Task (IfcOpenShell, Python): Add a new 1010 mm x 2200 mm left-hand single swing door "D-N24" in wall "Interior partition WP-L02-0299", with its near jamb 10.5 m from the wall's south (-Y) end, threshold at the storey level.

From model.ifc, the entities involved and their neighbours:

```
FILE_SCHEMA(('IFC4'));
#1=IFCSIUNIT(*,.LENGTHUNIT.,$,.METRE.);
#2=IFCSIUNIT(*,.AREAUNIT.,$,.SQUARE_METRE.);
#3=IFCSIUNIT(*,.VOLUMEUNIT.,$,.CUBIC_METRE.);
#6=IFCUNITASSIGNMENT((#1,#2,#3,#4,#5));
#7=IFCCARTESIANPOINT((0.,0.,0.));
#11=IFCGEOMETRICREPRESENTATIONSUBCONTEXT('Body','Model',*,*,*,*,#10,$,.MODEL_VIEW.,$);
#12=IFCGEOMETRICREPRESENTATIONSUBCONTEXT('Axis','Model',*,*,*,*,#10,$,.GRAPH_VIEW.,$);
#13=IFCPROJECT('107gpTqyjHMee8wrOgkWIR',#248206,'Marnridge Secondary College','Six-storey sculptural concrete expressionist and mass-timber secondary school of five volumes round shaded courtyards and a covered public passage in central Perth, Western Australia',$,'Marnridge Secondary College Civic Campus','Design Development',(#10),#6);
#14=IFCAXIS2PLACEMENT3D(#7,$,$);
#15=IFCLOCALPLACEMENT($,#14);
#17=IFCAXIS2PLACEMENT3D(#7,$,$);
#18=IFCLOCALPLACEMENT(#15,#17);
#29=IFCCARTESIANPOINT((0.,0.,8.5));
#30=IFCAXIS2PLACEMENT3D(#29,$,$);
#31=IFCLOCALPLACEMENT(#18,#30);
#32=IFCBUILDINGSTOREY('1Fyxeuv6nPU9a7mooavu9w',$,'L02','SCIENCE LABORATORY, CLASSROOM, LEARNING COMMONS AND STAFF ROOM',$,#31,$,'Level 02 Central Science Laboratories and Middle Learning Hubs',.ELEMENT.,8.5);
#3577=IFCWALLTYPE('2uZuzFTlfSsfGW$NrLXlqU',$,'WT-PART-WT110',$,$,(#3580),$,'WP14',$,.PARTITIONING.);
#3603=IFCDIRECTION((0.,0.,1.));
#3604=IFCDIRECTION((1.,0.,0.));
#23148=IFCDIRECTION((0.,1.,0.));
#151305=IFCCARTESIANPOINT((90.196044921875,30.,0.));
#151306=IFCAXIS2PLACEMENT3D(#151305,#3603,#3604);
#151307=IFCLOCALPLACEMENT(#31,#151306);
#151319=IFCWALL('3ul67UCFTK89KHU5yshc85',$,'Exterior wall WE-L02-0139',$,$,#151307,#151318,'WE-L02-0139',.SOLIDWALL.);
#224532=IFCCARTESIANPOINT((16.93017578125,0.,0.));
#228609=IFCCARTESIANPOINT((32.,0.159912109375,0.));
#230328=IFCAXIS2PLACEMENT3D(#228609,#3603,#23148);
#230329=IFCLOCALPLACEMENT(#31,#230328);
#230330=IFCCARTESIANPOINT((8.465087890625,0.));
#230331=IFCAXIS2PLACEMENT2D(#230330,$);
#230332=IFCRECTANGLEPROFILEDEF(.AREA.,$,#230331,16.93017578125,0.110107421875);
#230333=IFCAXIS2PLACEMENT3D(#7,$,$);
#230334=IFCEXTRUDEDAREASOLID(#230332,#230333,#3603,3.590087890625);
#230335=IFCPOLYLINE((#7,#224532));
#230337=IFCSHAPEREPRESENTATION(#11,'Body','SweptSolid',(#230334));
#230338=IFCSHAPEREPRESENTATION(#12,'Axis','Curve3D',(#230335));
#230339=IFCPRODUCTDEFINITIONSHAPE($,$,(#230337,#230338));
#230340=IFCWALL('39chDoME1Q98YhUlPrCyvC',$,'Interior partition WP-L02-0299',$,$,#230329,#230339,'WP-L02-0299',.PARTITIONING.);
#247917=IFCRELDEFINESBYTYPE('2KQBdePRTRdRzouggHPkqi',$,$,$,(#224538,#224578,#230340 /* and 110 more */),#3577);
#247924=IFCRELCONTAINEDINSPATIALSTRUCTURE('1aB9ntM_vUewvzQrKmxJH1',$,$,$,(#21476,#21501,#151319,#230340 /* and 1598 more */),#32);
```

```python
import numpy as np
import ifcopenshell
import ifcopenshell.api.feature
import ifcopenshell.api.geometry
import ifcopenshell.api.root
import ifcopenshell.api.spatial
import ifcopenshell.geom
import ifcopenshell.util.element
import ifcopenshell.util.placement
import ifcopenshell.util.representation
import ifcopenshell.util.shape
import ifcopenshell.util.unit

model = ifcopenshell.open("model.ifc")
unit_scale = ifcopenshell.util.unit.calculate_unit_scale(model)
settings = ifcopenshell.geom.settings()


def volume(element):
    """Net volume in cubic metres, openings subtracted."""
    shape = ifcopenshell.geom.create_shape(settings, element)
    return ifcopenshell.util.shape.get_volume(shape.geometry)


wall = model.by_id(230340)
storey = ifcopenshell.util.element.get_container(wall, ifc_class="IfcBuildingStorey")
context = ifcopenshell.util.representation.get_context(model, "Model", "Body", "MODEL_VIEW")
before = volume(wall)

width, height, from_end, sill = 1.01, 2.2, 10.5, 0.0  # metres

# The wall runs along its own X axis, and the end named is its -X end.
wall_shape = ifcopenshell.geom.create_shape(settings, wall)
x, y, z = ifcopenshell.util.shape.get_vertices(wall_shape.geometry).T
start = x.min() + from_end
face, thickness = float(y.min()), float(y.max() - y.min())
wall_matrix = ifcopenshell.util.placement.get_local_placement(wall.ObjectPlacement)
level = ifcopenshell.util.placement.get_local_placement(storey.ObjectPlacement)[2, 3]


def in_wall(x, y):
    """Placement at x, y metres in the wall's axes, at sill height."""
    matrix = wall_matrix.copy()
    matrix[:, 3] = wall_matrix @ np.array([x / unit_scale, y / unit_scale, 0.0, 1.0])
    matrix[2, 3] = level + sill / unit_scale
    return matrix


# Opening: a box that overshoots both wall faces by 50 mm.
opening = ifcopenshell.api.root.create_entity(model, ifc_class="IfcOpeningElement", predefined_type="OPENING")
box = ifcopenshell.api.geometry.add_wall_representation(
    model, context=context, length=width, height=height, thickness=thickness + 0.1
)
ifcopenshell.api.geometry.assign_representation(model, product=opening, representation=box)
ifcopenshell.api.geometry.edit_object_placement(model, product=opening, matrix=in_wall(start, face - 0.05), is_si=False)
ifcopenshell.api.feature.add_feature(model, feature=opening, element=wall)

door = ifcopenshell.api.root.create_entity(model, ifc_class="IfcDoor", name="D-N24", predefined_type="DOOR")
door.OverallWidth, door.OverallHeight = width / unit_scale, height / unit_scale
door.OperationType = "SINGLE_SWING_LEFT"
body = ifcopenshell.api.geometry.add_door_representation(
    model,
    context=context,
    overall_width=door.OverallWidth,
    overall_height=door.OverallHeight,
    operation_type="SINGLE_SWING_LEFT",
    lining_properties={"LiningDepth": thickness / unit_scale, "ThresholdDepth": thickness / unit_scale},
)
ifcopenshell.api.geometry.assign_representation(model, product=door, representation=body)
ifcopenshell.api.spatial.assign_container(model, products=[door], relating_structure=storey)
ifcopenshell.api.feature.add_filling(model, opening=opening, element=door)

# The lining spans the wall, so the door starts at the wall face.
ifcopenshell.api.geometry.edit_object_placement(model, product=door, matrix=in_wall(start, face), is_si=False)

after = volume(wall)

print(f"wall volume {before:.3f} -> {after:.3f} m3")

model.write("model_v2.ifc")
```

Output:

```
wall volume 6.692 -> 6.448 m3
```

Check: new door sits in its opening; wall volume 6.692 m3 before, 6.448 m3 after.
